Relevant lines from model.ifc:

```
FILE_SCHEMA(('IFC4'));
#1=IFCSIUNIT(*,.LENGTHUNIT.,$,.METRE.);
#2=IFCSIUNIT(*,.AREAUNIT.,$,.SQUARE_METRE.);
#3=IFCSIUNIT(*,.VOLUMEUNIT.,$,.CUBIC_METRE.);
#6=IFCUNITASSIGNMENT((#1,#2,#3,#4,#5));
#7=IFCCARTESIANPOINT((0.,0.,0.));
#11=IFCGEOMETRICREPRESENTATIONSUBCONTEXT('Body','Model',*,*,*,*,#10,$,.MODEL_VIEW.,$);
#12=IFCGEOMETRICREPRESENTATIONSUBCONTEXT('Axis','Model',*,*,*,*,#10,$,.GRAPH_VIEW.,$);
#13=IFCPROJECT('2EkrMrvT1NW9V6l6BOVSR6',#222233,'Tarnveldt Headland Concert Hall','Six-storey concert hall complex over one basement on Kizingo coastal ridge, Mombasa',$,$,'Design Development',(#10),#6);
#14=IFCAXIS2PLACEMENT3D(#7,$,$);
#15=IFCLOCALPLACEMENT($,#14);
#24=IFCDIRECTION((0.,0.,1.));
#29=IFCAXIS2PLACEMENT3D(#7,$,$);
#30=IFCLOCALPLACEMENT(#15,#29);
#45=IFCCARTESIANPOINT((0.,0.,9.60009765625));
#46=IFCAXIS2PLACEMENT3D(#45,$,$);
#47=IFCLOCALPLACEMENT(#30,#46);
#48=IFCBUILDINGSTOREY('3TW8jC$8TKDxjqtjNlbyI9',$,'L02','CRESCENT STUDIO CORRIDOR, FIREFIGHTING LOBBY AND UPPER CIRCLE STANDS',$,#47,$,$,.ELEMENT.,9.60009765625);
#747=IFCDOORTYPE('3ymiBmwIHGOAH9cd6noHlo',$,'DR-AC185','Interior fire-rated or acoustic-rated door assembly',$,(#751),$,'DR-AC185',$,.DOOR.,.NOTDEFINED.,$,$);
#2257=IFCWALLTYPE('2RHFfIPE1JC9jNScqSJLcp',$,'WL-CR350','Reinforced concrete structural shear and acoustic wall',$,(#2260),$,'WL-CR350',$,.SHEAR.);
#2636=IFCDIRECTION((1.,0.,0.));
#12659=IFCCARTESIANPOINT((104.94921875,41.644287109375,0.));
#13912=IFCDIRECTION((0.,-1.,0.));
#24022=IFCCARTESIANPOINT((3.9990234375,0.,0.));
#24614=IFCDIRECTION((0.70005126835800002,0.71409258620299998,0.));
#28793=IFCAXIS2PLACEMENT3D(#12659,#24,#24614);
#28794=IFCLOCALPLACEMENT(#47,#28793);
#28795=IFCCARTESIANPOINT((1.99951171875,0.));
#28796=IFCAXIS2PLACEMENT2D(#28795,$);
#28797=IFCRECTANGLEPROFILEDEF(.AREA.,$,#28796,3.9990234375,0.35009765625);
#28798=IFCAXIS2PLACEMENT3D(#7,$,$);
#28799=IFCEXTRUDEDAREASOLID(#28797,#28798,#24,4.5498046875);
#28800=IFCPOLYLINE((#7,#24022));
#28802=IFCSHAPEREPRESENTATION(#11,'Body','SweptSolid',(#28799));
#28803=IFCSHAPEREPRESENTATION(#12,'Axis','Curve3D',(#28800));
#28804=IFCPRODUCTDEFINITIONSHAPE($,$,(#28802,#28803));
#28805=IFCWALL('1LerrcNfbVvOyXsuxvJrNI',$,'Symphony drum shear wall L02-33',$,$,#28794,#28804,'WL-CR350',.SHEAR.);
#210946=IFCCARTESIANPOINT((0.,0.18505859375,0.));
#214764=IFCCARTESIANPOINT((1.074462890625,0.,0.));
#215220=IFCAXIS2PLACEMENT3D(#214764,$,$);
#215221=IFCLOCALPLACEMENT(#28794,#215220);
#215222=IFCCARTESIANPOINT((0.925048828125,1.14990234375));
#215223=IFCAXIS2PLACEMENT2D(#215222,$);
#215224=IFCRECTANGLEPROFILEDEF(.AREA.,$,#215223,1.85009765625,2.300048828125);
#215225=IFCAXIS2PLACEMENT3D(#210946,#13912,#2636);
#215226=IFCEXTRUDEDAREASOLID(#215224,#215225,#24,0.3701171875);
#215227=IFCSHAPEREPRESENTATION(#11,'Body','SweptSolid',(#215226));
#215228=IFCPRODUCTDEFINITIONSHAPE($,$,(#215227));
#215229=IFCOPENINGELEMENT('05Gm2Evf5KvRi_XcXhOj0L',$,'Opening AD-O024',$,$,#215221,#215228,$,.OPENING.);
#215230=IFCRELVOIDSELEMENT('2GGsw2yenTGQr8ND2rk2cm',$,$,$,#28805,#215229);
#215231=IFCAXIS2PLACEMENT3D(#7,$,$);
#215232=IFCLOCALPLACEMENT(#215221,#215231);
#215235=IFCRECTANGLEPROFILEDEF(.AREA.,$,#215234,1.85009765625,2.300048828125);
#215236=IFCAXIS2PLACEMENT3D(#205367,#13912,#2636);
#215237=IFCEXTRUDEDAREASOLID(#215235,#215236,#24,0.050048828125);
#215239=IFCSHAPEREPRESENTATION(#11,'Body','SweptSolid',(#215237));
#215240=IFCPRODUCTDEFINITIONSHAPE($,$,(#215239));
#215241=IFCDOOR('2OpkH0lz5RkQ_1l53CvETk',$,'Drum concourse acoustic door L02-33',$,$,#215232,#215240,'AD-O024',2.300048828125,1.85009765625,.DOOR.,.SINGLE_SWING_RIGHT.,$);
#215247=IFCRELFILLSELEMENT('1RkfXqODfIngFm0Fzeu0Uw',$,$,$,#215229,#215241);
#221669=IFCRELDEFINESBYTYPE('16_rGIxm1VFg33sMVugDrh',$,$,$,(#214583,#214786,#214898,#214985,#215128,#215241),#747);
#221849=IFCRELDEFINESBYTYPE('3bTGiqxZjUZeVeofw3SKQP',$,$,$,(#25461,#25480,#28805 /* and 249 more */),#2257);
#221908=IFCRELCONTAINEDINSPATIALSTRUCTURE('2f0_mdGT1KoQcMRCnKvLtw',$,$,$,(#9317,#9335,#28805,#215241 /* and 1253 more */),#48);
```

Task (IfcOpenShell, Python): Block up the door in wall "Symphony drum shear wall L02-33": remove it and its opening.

```python
import ifcopenshell
import ifcopenshell.api.feature
import ifcopenshell.api.root
import ifcopenshell.geom
import ifcopenshell.util.shape

model = ifcopenshell.open("model.ifc")
settings = ifcopenshell.geom.settings()


def volume(element):
    """Net volume in cubic metres, openings subtracted."""
    shape = ifcopenshell.geom.create_shape(settings, element)
    return ifcopenshell.util.shape.get_volume(shape.geometry)


door = model.by_guid("2OpkH0lz5RkQ_1l53CvETk")
opening = door.FillsVoids[0].RelatingOpeningElement
wall = opening.VoidsElements[0].RelatingBuildingElement
before = volume(wall)

ifcopenshell.api.root.remove_product(model, product=door)
ifcopenshell.api.feature.remove_feature(model, feature=opening)

after = volume(wall)

print(f"wall volume {before:.3f} -> {after:.3f} m3")

model.write("model_updated.ifc")
```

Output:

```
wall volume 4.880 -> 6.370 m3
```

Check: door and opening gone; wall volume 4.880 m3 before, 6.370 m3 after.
